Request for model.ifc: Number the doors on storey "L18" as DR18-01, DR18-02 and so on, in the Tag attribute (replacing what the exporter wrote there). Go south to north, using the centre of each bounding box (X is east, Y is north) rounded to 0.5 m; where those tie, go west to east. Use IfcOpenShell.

First a look at what the model holds.

```python
import ifcopenshell
import ifcopenshell.util.element
import ifcopenshell.util.placement

model = ifcopenshell.open("model.ifc")
print(model.schema)
storey = next(s for s in model.by_type("IfcBuildingStorey") if s.Name == "L18")
doors = [e for e in ifcopenshell.util.element.get_decomposition(storey) if e.is_a("IfcDoor")]
for e in sorted(doors, key=lambda e: e.id()):
    origin = ifcopenshell.util.placement.get_local_placement(e.ObjectPlacement)[:3, 3]
    print(e.id(), e.Tag, e.Name, origin.round(2) + 0.0, sep=" | ")
```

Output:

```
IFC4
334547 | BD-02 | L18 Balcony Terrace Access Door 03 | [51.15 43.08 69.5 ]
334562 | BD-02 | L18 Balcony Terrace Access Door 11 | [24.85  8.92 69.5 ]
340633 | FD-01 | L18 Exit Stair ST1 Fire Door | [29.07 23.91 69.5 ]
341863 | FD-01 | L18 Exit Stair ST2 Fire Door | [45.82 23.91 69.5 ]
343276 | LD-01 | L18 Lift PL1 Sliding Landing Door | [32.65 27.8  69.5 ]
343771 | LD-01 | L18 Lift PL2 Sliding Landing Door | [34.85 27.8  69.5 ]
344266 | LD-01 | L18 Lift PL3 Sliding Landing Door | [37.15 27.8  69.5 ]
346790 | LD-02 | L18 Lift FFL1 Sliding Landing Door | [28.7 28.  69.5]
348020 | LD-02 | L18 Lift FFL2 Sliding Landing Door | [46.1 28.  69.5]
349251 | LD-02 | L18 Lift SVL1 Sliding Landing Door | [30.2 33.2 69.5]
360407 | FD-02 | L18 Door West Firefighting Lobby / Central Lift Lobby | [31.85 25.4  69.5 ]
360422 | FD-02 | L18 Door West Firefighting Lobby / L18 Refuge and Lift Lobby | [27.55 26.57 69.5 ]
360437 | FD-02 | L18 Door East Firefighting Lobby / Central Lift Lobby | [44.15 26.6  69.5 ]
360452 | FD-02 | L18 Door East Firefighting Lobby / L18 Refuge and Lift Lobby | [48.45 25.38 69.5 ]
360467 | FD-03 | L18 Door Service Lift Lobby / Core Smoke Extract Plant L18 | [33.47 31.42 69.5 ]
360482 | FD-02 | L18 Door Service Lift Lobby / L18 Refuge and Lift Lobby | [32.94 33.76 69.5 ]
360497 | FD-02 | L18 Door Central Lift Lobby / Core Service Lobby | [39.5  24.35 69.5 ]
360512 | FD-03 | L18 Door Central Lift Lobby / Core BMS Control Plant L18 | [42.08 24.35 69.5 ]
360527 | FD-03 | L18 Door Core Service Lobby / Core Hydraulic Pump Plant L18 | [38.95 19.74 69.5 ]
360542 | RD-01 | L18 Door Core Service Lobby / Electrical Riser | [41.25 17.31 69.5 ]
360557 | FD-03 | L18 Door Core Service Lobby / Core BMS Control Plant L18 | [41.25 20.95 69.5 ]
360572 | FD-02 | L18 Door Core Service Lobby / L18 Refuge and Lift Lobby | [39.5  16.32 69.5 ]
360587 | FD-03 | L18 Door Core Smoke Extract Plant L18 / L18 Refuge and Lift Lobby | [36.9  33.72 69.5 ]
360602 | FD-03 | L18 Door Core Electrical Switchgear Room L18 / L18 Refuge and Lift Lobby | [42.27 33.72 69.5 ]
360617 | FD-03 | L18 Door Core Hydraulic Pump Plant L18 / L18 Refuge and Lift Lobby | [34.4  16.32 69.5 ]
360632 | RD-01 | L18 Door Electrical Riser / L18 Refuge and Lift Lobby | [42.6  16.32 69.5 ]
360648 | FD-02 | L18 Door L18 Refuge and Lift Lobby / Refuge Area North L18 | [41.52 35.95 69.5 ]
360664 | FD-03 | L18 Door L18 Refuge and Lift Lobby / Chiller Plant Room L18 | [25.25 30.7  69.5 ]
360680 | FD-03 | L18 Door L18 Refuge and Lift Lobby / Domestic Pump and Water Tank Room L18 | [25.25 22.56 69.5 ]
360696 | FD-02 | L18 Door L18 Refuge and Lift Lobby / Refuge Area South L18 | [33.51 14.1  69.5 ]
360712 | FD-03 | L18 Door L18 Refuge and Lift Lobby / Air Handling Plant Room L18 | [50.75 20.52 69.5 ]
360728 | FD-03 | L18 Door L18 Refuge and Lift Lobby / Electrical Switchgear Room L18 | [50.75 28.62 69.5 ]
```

```python
import ifcopenshell
import ifcopenshell.geom
import ifcopenshell.util.element
import ifcopenshell.util.shape

model = ifcopenshell.open("model.ifc")
settings = ifcopenshell.geom.settings()
settings.set("use-world-coords", True)


def centre(element):
    shape = ifcopenshell.geom.create_shape(settings, element)
    return ifcopenshell.util.shape.get_bbox_centroid(shape.geometry)


storey = next(s for s in model.by_type("IfcBuildingStorey") if s.Name == "L18")
doors = [e for e in ifcopenshell.util.element.get_decomposition(storey) if e.is_a("IfcDoor")]

# Insertion points can sit at a corner or the storey origin, so sort by the geometry (in metres).
centres = {e: centre(e) for e in doors}
doors.sort(key=lambda e: (round(centres[e][1] / 0.5), centres[e][0]))

for i, e in enumerate(doors, start=1):
    number = f"DR18-{i:02d}"
    e.Tag = number
    print(e.id(), number)

model.write("model_updated.ifc")
```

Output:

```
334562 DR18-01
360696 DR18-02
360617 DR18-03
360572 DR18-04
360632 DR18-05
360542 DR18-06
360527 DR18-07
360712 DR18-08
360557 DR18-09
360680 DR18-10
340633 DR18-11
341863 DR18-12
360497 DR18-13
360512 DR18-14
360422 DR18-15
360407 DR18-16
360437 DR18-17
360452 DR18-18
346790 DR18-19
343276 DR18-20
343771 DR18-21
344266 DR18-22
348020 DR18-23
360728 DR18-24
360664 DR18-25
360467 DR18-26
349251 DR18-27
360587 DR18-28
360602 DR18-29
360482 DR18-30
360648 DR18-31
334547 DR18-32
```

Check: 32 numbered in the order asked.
